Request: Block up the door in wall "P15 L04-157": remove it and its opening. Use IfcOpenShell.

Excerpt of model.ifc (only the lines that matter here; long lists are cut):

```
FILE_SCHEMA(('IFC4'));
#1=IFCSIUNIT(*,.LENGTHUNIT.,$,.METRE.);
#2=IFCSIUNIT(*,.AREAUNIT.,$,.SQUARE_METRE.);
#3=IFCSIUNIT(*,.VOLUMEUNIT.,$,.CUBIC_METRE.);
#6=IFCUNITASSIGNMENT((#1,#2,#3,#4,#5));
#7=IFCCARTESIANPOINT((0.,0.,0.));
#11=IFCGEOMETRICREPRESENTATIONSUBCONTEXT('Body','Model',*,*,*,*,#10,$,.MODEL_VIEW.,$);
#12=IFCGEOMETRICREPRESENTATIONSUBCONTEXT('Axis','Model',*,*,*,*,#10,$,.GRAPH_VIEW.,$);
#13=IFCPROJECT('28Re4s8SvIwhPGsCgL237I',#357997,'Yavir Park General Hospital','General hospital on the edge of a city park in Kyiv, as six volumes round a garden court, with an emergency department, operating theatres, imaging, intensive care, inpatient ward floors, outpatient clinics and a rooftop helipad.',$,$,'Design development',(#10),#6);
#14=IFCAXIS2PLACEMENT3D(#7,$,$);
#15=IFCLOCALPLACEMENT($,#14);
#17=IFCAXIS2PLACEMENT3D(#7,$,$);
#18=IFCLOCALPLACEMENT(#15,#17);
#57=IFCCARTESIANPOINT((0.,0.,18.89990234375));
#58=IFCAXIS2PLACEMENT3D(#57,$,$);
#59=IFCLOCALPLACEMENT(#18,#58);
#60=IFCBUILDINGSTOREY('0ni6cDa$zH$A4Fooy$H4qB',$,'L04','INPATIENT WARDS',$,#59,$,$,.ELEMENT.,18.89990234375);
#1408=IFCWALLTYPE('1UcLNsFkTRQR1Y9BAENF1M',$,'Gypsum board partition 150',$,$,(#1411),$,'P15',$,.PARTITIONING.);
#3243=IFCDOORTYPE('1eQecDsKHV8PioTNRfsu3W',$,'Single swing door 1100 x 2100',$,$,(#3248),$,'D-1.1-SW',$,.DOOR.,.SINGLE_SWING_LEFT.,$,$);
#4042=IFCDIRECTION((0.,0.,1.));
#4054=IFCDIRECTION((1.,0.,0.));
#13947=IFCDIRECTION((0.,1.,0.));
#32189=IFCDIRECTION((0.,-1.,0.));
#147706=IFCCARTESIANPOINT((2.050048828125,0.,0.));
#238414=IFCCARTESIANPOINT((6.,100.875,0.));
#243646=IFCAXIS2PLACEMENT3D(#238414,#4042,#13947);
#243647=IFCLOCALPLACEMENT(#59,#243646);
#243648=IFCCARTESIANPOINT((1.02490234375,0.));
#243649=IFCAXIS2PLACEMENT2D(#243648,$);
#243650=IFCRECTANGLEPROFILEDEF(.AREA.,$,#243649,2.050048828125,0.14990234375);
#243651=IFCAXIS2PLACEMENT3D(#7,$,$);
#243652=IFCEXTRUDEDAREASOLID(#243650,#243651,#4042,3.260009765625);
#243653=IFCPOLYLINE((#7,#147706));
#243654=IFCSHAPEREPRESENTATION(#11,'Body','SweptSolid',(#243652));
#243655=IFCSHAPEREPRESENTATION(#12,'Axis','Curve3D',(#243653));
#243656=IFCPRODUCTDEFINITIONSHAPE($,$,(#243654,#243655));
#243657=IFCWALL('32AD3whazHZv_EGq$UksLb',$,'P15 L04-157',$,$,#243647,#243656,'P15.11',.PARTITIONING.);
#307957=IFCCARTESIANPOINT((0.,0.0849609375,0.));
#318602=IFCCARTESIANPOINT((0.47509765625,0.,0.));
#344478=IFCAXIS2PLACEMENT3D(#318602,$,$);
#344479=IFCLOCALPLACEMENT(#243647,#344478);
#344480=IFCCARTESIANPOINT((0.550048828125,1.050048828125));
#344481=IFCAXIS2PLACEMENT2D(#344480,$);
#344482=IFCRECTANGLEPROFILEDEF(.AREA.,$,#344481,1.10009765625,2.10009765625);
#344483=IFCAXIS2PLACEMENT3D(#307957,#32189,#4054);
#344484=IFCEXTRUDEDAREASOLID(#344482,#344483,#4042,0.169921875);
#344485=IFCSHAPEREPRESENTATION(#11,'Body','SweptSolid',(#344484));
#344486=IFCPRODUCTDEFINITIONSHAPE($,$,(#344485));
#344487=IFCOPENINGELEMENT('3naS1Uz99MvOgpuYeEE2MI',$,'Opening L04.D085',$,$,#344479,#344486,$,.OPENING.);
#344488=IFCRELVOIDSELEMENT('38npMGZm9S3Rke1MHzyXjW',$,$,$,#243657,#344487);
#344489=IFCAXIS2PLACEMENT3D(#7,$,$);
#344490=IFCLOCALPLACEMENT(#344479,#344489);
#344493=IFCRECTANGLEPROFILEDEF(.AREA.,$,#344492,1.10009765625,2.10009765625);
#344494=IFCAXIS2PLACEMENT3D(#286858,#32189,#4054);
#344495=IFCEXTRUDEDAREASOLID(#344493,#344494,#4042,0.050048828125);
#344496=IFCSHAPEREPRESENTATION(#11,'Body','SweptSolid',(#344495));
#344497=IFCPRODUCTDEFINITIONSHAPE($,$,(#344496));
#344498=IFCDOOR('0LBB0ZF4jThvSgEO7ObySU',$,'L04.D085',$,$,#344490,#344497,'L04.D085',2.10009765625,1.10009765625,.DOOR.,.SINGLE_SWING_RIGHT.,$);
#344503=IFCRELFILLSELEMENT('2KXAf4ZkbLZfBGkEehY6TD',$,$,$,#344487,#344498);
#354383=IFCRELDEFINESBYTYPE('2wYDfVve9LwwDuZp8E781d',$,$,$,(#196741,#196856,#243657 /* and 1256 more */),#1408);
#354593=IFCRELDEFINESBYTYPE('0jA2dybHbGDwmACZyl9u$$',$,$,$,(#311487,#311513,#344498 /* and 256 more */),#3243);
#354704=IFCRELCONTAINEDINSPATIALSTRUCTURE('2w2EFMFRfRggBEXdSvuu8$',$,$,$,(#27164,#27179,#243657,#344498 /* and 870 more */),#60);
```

```python
import ifcopenshell
import ifcopenshell.api.feature
import ifcopenshell.api.root
import ifcopenshell.geom
import ifcopenshell.util.shape

model = ifcopenshell.open("model.ifc")
settings = ifcopenshell.geom.settings()


def volume(element):
    """Net volume in cubic metres, openings subtracted."""
    shape = ifcopenshell.geom.create_shape(settings, element)
    return ifcopenshell.util.shape.get_volume(shape.geometry)


door = model.by_guid("0LBB0ZF4jThvSgEO7ObySU")
opening = door.FillsVoids[0].RelatingOpeningElement
wall = opening.VoidsElements[0].RelatingBuildingElement
before = volume(wall)

ifcopenshell.api.root.remove_product(model, product=door)
ifcopenshell.api.feature.remove_feature(model, feature=opening)

after = volume(wall)

print(f"wall volume {before:.3f} -> {after:.3f} m3")

model.write("model-out.ifc")
```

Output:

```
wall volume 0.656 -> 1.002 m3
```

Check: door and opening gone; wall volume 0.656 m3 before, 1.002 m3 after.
